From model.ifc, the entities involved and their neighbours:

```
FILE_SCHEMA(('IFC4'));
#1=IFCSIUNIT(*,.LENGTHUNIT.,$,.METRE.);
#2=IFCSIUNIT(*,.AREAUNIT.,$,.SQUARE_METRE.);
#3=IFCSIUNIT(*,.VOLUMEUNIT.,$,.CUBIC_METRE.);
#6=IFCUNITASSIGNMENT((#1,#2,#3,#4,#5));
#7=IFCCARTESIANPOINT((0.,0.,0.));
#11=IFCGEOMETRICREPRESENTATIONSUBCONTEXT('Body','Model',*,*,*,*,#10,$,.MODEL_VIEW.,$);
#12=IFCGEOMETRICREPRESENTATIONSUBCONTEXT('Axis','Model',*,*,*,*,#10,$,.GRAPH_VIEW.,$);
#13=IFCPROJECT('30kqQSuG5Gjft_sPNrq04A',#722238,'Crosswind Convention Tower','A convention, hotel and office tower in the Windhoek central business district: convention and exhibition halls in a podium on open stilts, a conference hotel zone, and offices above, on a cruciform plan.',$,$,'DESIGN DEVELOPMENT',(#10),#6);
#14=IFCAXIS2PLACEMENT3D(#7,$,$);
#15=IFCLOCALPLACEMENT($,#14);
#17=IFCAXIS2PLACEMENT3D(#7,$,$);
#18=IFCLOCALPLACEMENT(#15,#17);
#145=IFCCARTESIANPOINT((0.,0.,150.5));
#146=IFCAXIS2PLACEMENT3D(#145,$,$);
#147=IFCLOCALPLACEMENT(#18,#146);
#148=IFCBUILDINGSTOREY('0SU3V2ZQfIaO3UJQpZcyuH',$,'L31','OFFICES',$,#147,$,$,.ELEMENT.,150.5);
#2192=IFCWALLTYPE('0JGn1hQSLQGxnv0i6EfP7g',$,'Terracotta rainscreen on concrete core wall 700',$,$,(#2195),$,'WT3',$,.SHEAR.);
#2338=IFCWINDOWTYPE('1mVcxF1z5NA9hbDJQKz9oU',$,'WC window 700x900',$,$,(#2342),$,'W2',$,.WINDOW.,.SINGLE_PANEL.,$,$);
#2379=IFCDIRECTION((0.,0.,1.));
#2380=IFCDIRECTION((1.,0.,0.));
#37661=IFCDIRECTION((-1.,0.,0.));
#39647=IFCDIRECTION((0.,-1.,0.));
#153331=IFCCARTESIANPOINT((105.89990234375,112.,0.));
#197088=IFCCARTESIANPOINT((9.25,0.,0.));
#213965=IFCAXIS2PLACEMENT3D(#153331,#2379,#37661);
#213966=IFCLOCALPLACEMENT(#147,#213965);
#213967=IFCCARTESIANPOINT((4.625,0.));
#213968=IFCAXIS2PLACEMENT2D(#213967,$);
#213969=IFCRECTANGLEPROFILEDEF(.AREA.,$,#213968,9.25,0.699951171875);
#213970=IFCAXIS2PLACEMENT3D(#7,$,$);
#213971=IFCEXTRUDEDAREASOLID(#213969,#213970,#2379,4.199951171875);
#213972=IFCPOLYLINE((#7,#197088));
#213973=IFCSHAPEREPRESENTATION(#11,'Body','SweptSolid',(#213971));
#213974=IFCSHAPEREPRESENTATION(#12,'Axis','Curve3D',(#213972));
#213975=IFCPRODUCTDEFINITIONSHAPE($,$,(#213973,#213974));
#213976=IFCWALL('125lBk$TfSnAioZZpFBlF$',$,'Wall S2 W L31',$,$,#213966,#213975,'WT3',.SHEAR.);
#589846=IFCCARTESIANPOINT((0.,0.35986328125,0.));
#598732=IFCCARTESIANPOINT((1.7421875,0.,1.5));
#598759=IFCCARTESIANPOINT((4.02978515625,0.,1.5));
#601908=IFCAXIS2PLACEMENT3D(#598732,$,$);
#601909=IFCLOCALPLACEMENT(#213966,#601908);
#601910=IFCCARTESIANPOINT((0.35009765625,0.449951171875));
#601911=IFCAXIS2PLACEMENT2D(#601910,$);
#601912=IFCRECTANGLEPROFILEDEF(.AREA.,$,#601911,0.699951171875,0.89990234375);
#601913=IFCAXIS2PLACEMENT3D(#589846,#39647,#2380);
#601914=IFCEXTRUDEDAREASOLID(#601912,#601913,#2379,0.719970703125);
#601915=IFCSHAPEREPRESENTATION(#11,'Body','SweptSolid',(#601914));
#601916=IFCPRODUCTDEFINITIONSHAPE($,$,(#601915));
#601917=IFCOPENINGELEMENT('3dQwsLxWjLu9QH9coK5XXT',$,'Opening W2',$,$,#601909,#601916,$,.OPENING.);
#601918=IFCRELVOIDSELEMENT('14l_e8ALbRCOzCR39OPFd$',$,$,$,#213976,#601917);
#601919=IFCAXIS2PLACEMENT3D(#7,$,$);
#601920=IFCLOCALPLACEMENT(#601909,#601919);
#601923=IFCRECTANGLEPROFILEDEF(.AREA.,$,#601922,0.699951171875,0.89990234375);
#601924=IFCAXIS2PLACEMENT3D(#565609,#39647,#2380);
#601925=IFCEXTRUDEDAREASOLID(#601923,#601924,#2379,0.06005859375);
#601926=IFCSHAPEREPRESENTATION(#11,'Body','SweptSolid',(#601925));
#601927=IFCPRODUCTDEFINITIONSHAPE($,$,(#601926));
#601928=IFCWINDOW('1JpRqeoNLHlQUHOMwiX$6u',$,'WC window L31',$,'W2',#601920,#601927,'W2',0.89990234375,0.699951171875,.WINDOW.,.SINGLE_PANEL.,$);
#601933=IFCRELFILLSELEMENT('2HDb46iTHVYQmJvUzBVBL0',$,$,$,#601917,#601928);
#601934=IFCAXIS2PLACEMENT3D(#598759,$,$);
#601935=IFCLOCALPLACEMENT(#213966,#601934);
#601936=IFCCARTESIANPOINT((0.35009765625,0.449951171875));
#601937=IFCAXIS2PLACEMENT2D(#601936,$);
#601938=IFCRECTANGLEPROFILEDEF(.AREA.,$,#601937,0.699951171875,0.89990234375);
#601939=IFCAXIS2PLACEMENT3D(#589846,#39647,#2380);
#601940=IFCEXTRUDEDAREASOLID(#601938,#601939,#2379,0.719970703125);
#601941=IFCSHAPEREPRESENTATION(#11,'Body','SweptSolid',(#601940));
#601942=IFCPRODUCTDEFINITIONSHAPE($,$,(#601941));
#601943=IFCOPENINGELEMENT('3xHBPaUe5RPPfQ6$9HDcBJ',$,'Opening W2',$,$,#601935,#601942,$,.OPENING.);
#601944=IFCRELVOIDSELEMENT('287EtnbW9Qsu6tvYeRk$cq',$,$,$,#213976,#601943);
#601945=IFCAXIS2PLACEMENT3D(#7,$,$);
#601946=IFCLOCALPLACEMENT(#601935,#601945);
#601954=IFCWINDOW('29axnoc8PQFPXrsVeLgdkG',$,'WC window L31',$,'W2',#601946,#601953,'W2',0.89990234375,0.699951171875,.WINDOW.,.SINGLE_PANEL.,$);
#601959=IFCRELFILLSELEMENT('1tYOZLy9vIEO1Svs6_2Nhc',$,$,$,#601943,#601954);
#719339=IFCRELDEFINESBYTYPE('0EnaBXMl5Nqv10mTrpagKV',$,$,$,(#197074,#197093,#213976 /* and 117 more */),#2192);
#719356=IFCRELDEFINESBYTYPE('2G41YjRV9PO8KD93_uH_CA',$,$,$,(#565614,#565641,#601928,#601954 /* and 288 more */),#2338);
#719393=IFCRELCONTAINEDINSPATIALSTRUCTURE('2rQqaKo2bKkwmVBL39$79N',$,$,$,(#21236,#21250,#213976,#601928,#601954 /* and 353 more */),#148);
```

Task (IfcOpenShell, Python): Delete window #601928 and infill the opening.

```python
import ifcopenshell
import ifcopenshell.api.feature
import ifcopenshell.api.root
import ifcopenshell.geom
import ifcopenshell.util.shape

model = ifcopenshell.open("model.ifc")
settings = ifcopenshell.geom.settings()


def volume(element):
    """Net volume in cubic metres, openings subtracted."""
    shape = ifcopenshell.geom.create_shape(settings, element)
    return ifcopenshell.util.shape.get_volume(shape.geometry)


window = model.by_guid("1JpRqeoNLHlQUHOMwiX$6u")
opening = window.FillsVoids[0].RelatingOpeningElement
wall = opening.VoidsElements[0].RelatingBuildingElement
before = volume(wall)

ifcopenshell.api.root.remove_product(model, product=window)
ifcopenshell.api.feature.remove_feature(model, feature=opening)

after = volume(wall)

print(f"wall volume {before:.3f} -> {after:.3f} m3")

model.write("model_rev.ifc")
```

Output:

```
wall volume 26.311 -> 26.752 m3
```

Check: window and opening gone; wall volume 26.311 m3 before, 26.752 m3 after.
